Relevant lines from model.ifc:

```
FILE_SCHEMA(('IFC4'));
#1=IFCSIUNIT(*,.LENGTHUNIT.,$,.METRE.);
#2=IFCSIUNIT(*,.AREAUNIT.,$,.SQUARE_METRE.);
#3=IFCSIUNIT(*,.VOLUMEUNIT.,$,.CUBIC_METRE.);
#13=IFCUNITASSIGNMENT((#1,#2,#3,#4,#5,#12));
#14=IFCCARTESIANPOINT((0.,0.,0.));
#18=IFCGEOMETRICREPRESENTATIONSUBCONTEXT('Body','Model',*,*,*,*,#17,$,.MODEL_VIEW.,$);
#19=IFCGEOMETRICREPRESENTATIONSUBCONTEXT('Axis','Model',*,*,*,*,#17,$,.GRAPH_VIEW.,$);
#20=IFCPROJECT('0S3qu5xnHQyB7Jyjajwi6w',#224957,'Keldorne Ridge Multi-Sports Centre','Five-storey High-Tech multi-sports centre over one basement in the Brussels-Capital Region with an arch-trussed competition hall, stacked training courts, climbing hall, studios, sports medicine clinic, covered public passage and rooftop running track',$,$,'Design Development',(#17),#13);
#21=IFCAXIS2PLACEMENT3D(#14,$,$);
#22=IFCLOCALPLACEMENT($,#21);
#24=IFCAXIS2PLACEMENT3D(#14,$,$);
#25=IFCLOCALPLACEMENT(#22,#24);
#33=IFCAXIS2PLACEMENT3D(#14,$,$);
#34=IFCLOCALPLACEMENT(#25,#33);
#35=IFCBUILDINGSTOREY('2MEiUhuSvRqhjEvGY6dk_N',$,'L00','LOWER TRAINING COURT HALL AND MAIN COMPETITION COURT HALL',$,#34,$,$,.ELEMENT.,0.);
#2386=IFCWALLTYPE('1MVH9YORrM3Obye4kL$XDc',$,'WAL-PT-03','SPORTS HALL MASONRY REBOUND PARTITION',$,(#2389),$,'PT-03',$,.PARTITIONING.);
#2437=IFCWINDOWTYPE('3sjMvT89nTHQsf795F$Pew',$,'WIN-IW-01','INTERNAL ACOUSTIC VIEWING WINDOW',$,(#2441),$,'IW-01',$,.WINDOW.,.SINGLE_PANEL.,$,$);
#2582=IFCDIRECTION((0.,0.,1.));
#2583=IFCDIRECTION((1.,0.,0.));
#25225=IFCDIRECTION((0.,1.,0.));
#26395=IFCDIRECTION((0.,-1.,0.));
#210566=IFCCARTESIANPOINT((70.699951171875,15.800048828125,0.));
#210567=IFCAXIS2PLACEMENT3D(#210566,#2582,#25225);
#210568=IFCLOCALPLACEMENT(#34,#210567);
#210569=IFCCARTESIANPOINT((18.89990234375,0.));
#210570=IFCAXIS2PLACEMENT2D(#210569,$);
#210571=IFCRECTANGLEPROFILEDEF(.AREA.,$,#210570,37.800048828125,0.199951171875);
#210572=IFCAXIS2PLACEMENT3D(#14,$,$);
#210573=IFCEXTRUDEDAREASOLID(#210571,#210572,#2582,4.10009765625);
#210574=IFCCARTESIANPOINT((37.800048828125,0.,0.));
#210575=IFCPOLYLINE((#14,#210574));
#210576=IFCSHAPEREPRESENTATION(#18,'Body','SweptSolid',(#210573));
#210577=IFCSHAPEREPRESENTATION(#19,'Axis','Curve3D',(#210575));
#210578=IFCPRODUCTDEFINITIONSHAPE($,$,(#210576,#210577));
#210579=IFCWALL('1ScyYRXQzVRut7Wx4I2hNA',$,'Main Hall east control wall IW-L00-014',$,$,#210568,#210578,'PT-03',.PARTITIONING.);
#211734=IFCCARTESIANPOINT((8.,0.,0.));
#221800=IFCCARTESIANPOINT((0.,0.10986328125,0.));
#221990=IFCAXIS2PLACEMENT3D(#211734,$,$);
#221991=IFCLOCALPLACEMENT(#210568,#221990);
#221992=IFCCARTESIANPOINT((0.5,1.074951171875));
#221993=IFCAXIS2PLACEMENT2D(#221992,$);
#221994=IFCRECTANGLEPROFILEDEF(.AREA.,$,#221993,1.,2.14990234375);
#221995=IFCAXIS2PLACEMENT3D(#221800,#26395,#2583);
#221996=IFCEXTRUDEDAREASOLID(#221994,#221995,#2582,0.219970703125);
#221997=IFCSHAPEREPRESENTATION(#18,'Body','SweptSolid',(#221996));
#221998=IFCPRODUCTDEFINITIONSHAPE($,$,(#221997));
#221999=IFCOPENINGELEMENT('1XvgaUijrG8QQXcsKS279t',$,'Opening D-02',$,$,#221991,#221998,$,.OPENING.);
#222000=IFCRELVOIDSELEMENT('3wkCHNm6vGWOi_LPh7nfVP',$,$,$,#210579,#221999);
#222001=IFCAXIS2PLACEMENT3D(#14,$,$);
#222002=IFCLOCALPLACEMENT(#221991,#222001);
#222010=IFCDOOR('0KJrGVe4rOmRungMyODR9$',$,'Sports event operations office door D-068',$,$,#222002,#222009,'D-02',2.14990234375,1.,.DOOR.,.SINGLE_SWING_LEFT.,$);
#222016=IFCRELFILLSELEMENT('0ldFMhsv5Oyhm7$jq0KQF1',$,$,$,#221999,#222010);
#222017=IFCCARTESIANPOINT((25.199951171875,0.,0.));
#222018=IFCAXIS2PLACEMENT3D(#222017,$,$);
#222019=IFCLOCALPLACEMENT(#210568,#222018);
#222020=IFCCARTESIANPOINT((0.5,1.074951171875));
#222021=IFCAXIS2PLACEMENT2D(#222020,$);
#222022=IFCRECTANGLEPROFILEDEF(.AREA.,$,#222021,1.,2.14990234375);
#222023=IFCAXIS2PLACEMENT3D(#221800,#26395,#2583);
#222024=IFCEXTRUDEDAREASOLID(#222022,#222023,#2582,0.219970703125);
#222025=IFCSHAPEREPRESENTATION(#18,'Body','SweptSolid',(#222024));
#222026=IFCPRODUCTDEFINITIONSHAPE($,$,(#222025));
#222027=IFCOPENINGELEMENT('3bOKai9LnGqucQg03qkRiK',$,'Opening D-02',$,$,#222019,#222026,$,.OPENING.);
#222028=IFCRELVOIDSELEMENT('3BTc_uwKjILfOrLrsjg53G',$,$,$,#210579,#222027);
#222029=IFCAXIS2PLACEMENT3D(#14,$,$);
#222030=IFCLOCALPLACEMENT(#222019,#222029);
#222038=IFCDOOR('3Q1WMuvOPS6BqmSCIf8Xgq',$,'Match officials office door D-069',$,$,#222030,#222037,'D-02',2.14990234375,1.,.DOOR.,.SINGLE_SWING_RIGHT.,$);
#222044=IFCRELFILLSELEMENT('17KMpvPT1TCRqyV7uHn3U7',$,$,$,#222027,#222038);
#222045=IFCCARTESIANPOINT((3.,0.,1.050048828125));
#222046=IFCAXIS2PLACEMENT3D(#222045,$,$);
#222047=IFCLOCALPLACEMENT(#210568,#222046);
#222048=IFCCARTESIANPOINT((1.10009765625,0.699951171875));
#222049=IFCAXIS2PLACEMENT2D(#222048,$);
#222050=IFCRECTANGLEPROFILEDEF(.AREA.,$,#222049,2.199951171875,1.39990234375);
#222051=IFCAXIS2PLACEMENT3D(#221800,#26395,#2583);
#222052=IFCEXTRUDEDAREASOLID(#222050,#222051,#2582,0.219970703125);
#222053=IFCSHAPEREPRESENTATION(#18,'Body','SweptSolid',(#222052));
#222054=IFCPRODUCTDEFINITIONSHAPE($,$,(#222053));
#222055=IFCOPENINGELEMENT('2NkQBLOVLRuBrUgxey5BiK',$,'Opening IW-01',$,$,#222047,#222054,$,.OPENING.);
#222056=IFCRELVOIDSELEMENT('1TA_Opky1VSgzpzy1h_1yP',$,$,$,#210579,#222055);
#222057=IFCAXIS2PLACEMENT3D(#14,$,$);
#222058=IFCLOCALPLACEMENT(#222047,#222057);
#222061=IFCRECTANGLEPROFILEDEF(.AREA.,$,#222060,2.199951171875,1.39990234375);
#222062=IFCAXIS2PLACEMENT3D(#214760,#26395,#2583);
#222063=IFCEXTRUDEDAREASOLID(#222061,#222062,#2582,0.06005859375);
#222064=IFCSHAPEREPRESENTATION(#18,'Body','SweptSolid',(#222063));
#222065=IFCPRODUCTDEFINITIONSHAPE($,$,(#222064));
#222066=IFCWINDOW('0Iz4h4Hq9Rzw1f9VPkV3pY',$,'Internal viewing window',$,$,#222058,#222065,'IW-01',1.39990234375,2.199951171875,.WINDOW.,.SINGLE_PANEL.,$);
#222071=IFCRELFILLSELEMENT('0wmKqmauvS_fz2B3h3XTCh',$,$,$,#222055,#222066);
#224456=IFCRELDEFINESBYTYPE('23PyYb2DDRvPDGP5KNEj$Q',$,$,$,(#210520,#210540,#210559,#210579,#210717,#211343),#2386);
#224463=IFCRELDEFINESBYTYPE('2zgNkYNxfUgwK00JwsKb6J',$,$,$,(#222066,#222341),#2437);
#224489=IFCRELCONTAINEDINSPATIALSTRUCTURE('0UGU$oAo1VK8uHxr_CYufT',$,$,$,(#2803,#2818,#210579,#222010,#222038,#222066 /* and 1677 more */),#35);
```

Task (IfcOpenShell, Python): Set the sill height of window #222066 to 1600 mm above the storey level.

```python
import numpy as np
import ifcopenshell
import ifcopenshell.api.geometry
import ifcopenshell.geom
import ifcopenshell.util.element
import ifcopenshell.util.placement
import ifcopenshell.util.shape
import ifcopenshell.util.unit

model = ifcopenshell.open("model.ifc")
unit_scale = ifcopenshell.util.unit.calculate_unit_scale(model)

window = model.by_guid("0Iz4h4Hq9Rzw1f9VPkV3pY")
opening = window.FillsVoids[0].RelatingOpeningElement
storey = ifcopenshell.util.element.get_container(window, ifc_class="IfcBuildingStorey")
level = ifcopenshell.util.placement.get_local_placement(storey.ObjectPlacement)[2, 3]

# The opening's origin need not be at the sill, so measure its lowest point.
shape = ifcopenshell.geom.create_shape(ifcopenshell.geom.settings(), opening)
bottom = ifcopenshell.util.shape.get_shape_bottom_elevation(shape, shape.geometry) / unit_scale
dz = level + 1.6 / unit_scale - bottom

shift = np.array([0.0, 0.0, dz])
# The window is placed relative to its opening, so it follows when the opening moves.
matrix = ifcopenshell.util.placement.get_local_placement(opening.ObjectPlacement)
matrix[:3, 3] += shift
ifcopenshell.api.geometry.edit_object_placement(
    model, product=opening, matrix=matrix, is_si=False, should_transform_children=True
)

print(f"moved by {dz * unit_scale:+.3f} m")

model.write("model-out.ifc")
```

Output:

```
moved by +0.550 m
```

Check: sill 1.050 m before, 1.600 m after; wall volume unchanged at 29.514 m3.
